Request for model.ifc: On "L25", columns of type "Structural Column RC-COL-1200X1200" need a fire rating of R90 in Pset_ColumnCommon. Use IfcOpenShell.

First a look at what the model holds.

```python
import ifcopenshell
import ifcopenshell.util.element

model = ifcopenshell.open("model.ifc")
print(model.schema)
storey = next(s for s in model.by_type("IfcBuildingStorey") if s.Name == "L25")
columns = [e for e in ifcopenshell.util.element.get_decomposition(storey) if e.is_a("IfcColumn")]
seen = {}
for e in columns:
    element_type = ifcopenshell.util.element.get_type(e)
    key = (element_type.Name if element_type != e and element_type else None, ifcopenshell.util.element.get_pset(e, "Pset_ColumnCommon", "FireRating"))
    seen[key] = seen.get(key, 0) + 1
for (name, value), count in sorted(seen.items(), key=str):
    print(count, "x", name, "|", value)
```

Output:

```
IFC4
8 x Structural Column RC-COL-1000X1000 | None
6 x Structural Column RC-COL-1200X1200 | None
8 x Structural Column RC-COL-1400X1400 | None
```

```python
import ifcopenshell
import ifcopenshell.api.pset
import ifcopenshell.util.element

model = ifcopenshell.open("model.ifc")

storey = next(s for s in model.by_type("IfcBuildingStorey") if s.Name == "L25")
columns = [e for e in ifcopenshell.util.element.get_decomposition(storey) if e.is_a("IfcColumn")]

count = 0
for e in columns:
    element_type = ifcopenshell.util.element.get_type(e)
    if element_type in (None, e) or element_type.Name != "Structural Column RC-COL-1200X1200":
        continue
    found = ifcopenshell.util.element.get_pset(e, "Pset_ColumnCommon", should_inherit=False)
    if found:
        pset = model.by_id(found["id"])
        if len(ifcopenshell.util.element.get_elements_by_pset(pset)) > 1:
            pset = ifcopenshell.api.pset.unshare_pset(model, products=[e], pset=pset)[0]
    else:
        pset = ifcopenshell.api.pset.add_pset(model, product=e, name="Pset_ColumnCommon")
    ifcopenshell.api.pset.edit_pset(model, pset=pset, properties={"FireRating": "R90"})
    count += 1

print(count, "columns updated")

model.write("model_updated.ifc")
```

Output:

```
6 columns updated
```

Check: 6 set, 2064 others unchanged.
